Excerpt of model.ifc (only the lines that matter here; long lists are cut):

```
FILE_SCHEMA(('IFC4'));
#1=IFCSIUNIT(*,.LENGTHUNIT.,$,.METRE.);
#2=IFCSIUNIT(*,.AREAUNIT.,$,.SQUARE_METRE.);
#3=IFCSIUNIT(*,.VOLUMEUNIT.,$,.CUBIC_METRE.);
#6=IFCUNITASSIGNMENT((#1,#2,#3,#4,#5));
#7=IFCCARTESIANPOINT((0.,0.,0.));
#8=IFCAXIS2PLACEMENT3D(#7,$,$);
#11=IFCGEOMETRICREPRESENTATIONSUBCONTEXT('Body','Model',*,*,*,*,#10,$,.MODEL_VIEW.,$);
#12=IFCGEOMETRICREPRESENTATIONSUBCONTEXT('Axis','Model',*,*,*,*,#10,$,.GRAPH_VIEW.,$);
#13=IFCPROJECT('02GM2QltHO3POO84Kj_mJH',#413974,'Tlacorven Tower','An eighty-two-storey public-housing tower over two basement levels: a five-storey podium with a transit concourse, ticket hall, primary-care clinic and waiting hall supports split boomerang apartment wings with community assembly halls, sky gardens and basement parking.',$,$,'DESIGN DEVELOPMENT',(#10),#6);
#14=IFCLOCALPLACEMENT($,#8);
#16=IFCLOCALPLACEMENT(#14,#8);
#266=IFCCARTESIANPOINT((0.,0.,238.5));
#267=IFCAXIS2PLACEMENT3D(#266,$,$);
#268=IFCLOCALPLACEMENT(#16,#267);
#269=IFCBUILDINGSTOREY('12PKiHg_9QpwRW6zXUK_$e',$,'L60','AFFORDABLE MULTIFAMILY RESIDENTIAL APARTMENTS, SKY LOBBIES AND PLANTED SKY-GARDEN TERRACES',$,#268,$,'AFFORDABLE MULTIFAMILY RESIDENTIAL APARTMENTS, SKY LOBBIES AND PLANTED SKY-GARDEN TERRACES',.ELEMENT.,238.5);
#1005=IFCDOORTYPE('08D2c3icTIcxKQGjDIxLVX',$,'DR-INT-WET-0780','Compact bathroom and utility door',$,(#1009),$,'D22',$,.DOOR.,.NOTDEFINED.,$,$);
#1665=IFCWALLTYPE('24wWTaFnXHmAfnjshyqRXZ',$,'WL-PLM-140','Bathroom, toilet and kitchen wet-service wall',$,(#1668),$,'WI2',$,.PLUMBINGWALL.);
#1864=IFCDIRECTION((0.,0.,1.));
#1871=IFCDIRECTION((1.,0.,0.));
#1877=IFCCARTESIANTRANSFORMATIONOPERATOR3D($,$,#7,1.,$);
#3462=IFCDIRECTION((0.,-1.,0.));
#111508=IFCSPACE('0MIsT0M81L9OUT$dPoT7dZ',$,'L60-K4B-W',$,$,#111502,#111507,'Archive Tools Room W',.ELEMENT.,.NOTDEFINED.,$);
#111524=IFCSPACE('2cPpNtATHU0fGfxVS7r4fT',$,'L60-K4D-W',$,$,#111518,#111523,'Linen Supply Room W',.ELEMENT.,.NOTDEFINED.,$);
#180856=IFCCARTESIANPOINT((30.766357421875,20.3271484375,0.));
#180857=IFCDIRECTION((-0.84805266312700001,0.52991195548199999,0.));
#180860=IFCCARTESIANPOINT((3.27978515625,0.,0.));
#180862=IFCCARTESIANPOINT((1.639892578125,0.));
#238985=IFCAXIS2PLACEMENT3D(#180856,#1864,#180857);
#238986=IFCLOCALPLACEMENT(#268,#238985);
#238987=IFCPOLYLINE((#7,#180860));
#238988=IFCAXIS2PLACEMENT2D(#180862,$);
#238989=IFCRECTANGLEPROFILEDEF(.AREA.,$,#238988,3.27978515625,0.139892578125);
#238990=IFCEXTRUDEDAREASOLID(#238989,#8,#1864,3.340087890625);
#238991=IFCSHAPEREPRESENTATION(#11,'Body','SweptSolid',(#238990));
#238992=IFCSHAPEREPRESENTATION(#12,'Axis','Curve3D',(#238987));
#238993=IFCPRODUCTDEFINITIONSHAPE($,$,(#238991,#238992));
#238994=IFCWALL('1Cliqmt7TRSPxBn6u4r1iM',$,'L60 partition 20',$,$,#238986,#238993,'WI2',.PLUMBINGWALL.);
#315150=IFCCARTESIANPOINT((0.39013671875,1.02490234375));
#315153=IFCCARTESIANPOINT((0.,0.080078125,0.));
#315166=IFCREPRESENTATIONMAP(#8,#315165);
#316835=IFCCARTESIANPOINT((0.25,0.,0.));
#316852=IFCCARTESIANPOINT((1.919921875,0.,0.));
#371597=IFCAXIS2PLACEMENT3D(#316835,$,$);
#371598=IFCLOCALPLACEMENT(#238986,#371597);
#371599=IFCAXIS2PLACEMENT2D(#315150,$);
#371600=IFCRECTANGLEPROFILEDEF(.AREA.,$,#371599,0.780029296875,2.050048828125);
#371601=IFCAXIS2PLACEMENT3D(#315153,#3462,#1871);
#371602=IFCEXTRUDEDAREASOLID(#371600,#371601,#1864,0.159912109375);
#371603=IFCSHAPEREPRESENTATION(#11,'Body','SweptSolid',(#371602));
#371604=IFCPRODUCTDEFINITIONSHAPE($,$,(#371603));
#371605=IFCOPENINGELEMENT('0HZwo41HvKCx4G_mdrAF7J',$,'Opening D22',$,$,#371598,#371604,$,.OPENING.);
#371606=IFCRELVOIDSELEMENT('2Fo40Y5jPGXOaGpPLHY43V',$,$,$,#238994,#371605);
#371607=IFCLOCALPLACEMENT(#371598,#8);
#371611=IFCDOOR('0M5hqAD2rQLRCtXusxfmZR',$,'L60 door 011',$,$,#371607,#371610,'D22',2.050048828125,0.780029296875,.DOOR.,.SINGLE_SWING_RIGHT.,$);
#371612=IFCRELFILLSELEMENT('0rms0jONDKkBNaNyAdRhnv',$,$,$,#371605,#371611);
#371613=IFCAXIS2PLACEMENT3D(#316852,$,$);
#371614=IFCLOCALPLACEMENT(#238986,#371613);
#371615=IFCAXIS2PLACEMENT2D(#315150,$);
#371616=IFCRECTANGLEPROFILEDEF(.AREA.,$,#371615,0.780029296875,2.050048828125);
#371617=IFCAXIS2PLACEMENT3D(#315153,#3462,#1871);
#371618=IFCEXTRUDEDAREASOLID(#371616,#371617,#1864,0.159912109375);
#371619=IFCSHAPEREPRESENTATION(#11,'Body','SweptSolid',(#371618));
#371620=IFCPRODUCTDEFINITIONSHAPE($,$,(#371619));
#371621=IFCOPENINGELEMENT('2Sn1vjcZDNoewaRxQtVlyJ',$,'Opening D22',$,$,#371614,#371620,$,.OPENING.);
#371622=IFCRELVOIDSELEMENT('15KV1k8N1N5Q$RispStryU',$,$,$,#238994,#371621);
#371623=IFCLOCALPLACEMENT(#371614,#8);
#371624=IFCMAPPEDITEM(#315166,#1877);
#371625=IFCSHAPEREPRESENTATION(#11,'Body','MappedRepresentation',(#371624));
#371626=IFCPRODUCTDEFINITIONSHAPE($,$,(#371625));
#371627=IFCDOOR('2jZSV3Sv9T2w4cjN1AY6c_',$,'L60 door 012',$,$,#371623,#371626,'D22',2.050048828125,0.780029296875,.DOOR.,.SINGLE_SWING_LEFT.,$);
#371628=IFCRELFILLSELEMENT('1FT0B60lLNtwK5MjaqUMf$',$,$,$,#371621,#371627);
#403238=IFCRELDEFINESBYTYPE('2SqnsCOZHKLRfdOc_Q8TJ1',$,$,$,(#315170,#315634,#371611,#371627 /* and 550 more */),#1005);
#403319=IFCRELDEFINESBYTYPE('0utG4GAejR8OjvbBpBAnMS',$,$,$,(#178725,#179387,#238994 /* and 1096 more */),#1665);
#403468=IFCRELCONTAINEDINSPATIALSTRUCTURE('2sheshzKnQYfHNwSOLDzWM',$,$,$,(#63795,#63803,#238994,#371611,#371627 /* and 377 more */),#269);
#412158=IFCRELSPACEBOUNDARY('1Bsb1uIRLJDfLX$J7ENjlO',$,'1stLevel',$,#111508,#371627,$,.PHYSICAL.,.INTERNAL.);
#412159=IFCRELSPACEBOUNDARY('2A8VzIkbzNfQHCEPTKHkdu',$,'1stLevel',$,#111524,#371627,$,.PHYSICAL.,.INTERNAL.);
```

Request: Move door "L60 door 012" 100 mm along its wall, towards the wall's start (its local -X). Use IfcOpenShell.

```python
import ifcopenshell
import ifcopenshell.api.geometry
import ifcopenshell.util.placement
import ifcopenshell.util.unit

model = ifcopenshell.open("model.ifc")
unit_scale = ifcopenshell.util.unit.calculate_unit_scale(model)

door = model.by_guid("2jZSV3Sv9T2w4cjN1AY6c_")
opening = door.FillsVoids[0].RelatingOpeningElement
wall = opening.VoidsElements[0].RelatingBuildingElement

wall_matrix = ifcopenshell.util.placement.get_local_placement(wall.ObjectPlacement)
shift = wall_matrix[:3, 0] * -0.1 / unit_scale
before = ifcopenshell.util.placement.get_local_placement(door.ObjectPlacement)[:3, 3].copy()

# The door is placed relative to its opening, so it follows when the opening moves.
matrix = ifcopenshell.util.placement.get_local_placement(opening.ObjectPlacement)
matrix[:3, 3] += shift
ifcopenshell.api.geometry.edit_object_placement(
    model, product=opening, matrix=matrix, is_si=False, should_transform_children=True
)

after = ifcopenshell.util.placement.get_local_placement(door.ObjectPlacement)[:3, 3]
print("door moved by", (after - before).round(3) + 0.0)

model.write("model_v2.ifc")
```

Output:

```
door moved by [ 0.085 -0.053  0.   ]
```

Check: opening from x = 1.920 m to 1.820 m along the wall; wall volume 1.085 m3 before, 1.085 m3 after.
